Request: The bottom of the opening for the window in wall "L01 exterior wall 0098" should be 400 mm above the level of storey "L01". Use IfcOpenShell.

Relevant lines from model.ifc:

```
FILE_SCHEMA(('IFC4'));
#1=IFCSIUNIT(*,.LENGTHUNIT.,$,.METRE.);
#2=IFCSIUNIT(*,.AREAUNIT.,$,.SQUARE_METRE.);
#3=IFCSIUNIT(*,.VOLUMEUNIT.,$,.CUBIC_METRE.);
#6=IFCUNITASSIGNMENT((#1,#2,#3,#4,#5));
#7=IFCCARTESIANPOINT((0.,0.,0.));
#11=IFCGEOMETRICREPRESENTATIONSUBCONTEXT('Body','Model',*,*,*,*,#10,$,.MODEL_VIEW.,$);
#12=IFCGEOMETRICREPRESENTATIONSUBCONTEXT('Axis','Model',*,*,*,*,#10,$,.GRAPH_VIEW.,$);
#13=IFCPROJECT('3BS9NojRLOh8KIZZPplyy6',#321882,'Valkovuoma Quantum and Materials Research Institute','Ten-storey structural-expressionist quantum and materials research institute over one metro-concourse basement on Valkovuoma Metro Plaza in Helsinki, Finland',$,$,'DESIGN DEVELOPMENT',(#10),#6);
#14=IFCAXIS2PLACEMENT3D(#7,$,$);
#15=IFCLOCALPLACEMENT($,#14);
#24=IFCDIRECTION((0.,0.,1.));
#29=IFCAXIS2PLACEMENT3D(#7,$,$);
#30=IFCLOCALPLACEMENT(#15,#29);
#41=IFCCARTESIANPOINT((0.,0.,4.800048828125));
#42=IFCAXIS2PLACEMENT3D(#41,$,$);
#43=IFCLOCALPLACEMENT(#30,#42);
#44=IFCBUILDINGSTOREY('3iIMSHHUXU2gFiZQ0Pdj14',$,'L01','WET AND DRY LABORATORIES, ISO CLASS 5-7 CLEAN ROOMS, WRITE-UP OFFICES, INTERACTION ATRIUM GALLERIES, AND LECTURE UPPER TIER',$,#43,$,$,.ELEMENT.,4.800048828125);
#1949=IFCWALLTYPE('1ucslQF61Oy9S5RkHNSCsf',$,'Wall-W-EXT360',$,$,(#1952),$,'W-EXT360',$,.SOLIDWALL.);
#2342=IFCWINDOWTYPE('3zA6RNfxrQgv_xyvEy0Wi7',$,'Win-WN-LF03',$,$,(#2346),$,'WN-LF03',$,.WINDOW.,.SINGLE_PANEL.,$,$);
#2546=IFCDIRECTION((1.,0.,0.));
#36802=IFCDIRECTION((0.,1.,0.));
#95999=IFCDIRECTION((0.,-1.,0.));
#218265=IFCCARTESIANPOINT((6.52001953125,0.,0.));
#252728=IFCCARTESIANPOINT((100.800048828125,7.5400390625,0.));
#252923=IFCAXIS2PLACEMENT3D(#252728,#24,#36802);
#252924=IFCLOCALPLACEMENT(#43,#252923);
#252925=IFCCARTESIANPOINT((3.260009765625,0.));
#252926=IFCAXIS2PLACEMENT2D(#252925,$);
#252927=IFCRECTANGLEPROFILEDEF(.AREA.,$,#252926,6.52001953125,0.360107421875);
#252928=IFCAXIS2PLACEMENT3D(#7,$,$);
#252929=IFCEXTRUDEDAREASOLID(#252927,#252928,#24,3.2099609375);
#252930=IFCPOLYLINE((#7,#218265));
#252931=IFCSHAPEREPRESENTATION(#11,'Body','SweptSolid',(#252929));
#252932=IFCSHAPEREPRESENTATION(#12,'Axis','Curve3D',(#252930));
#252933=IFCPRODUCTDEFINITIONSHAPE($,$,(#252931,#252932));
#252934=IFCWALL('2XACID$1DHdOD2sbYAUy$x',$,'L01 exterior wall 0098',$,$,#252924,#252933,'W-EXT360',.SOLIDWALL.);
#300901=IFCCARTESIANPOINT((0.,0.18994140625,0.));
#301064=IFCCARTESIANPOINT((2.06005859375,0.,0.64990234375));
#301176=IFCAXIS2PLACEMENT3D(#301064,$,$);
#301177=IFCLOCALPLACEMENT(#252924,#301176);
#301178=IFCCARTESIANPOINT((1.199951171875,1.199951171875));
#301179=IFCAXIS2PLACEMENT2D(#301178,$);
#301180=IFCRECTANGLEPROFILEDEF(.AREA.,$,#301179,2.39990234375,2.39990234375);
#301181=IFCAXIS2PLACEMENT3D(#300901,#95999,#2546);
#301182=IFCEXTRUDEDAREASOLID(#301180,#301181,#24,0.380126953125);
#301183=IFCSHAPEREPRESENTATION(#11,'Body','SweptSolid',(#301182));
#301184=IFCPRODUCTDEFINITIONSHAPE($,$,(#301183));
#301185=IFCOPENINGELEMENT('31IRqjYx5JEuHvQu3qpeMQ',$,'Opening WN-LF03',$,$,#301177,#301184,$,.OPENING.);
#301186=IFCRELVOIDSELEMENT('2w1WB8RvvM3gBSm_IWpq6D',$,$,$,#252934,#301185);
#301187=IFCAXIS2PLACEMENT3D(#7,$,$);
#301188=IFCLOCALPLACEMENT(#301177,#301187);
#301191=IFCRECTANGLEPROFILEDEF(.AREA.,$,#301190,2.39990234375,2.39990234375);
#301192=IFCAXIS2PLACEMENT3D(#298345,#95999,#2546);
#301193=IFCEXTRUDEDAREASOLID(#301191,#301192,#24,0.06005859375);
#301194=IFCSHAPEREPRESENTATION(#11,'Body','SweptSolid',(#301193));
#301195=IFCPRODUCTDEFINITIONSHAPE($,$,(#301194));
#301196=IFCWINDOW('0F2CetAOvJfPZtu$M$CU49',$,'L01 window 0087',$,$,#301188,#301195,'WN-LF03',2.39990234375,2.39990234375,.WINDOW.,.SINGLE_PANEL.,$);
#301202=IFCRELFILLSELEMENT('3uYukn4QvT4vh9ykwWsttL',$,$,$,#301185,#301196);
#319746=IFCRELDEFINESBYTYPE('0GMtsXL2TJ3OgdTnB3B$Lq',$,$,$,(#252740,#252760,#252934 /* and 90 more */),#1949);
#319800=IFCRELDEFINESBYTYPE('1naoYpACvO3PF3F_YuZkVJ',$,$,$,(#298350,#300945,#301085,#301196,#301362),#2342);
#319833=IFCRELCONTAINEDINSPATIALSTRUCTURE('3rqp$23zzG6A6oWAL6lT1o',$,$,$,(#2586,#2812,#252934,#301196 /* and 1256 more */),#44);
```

```python
import numpy as np
import ifcopenshell
import ifcopenshell.api.geometry
import ifcopenshell.geom
import ifcopenshell.util.element
import ifcopenshell.util.placement
import ifcopenshell.util.shape
import ifcopenshell.util.unit

model = ifcopenshell.open("model.ifc")
unit_scale = ifcopenshell.util.unit.calculate_unit_scale(model)

window = model.by_guid("0F2CetAOvJfPZtu$M$CU49")
opening = window.FillsVoids[0].RelatingOpeningElement
storey = ifcopenshell.util.element.get_container(window, ifc_class="IfcBuildingStorey")
level = ifcopenshell.util.placement.get_local_placement(storey.ObjectPlacement)[2, 3]

# The opening's origin need not be at the sill, so measure its lowest point.
shape = ifcopenshell.geom.create_shape(ifcopenshell.geom.settings(), opening)
bottom = ifcopenshell.util.shape.get_shape_bottom_elevation(shape, shape.geometry) / unit_scale
dz = level + 0.4 - bottom

shift = np.array([0.0, 0.0, dz])
# The window is placed relative to its opening, so it follows when the opening moves.
matrix = ifcopenshell.util.placement.get_local_placement(opening.ObjectPlacement)
matrix[:3, 3] += shift
ifcopenshell.api.geometry.edit_object_placement(
    model, product=opening, matrix=matrix, is_si=False, should_transform_children=True
)

print(f"moved by {dz * unit_scale:+.3f} m")

model.write("model-out.ifc")
```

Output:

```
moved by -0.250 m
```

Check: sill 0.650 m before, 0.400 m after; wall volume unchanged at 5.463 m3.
